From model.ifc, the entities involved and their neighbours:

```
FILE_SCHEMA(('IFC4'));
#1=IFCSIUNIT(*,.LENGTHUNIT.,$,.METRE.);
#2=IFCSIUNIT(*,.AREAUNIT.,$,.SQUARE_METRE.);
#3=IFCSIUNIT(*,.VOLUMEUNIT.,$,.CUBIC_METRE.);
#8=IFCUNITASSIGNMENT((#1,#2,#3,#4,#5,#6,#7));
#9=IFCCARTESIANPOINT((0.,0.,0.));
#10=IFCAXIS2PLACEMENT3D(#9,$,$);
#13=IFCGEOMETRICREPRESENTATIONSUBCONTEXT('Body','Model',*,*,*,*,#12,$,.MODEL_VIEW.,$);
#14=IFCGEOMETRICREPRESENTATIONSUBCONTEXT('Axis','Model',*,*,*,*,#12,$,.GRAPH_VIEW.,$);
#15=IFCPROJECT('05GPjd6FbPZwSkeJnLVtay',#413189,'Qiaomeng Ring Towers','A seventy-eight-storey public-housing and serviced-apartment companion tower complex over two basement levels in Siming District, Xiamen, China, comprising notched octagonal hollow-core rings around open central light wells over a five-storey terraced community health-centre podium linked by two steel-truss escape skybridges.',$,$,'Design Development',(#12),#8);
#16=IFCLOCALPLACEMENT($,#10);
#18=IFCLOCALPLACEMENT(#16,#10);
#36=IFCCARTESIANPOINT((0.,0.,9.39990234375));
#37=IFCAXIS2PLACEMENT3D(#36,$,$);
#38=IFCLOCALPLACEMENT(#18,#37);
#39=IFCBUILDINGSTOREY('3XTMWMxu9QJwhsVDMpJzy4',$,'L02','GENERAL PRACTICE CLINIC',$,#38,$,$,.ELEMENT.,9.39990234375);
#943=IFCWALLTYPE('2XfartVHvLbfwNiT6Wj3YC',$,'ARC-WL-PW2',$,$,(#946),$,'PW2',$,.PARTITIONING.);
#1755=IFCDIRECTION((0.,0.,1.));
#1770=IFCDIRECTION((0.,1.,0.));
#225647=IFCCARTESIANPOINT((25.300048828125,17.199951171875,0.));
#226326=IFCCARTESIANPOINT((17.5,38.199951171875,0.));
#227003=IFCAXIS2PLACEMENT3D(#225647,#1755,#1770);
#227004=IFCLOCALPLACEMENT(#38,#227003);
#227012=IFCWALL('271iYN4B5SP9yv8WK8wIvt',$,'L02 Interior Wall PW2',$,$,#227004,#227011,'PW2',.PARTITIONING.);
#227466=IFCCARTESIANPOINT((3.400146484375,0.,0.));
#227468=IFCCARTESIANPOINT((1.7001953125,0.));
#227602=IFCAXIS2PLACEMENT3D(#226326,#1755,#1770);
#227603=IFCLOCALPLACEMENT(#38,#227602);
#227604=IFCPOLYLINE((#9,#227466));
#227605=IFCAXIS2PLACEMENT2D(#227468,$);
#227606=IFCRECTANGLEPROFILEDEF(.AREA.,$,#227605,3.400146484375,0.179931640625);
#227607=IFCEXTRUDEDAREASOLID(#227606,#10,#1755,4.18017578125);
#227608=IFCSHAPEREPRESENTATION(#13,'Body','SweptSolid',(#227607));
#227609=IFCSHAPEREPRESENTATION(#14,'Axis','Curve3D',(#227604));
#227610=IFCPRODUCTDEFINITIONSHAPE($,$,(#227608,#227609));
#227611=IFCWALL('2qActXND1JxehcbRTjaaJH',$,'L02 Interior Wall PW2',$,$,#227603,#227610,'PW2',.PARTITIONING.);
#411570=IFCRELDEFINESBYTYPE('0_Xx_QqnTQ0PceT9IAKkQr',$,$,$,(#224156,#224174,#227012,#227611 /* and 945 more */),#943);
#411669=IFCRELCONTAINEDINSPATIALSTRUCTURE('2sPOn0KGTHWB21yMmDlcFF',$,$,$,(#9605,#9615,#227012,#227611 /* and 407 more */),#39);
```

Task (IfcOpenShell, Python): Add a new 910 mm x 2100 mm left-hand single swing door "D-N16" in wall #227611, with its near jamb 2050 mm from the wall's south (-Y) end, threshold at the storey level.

```python
import numpy as np
import ifcopenshell
import ifcopenshell.api.feature
import ifcopenshell.api.geometry
import ifcopenshell.api.root
import ifcopenshell.api.spatial
import ifcopenshell.geom
import ifcopenshell.util.element
import ifcopenshell.util.placement
import ifcopenshell.util.representation
import ifcopenshell.util.shape
import ifcopenshell.util.unit

model = ifcopenshell.open("model.ifc")
unit_scale = ifcopenshell.util.unit.calculate_unit_scale(model)
settings = ifcopenshell.geom.settings()


def volume(element):
    """Net volume in cubic metres, openings subtracted."""
    shape = ifcopenshell.geom.create_shape(settings, element)
    return ifcopenshell.util.shape.get_volume(shape.geometry)


wall = model.by_id(227611)
storey = ifcopenshell.util.element.get_container(wall, ifc_class="IfcBuildingStorey")
context = ifcopenshell.util.representation.get_context(model, "Model", "Body", "MODEL_VIEW")
before = volume(wall)

width, height, from_end, sill = 0.91, 2.1, 2.05, 0.0  # metres

# The wall runs along its own X axis, and the end named is its -X end.
wall_shape = ifcopenshell.geom.create_shape(settings, wall)
x, y, z = ifcopenshell.util.shape.get_vertices(wall_shape.geometry).T
start = x.min() + from_end
face, thickness = float(y.min()), float(y.max() - y.min())
wall_matrix = ifcopenshell.util.placement.get_local_placement(wall.ObjectPlacement)
level = ifcopenshell.util.placement.get_local_placement(storey.ObjectPlacement)[2, 3]


def in_wall(x, y):
    """Placement at x, y metres in the wall's axes, at sill height."""
    matrix = wall_matrix.copy()
    matrix[:, 3] = wall_matrix @ np.array([x / unit_scale, y / unit_scale, 0.0, 1.0])
    matrix[2, 3] = level + sill / unit_scale
    return matrix


# Opening: a box that overshoots both wall faces by 50 mm.
opening = ifcopenshell.api.root.create_entity(model, ifc_class="IfcOpeningElement", predefined_type="OPENING")
box = ifcopenshell.api.geometry.add_wall_representation(
    model, context=context, length=width, height=height, thickness=thickness + 0.1
)
ifcopenshell.api.geometry.assign_representation(model, product=opening, representation=box)
ifcopenshell.api.geometry.edit_object_placement(model, product=opening, matrix=in_wall(start, face - 0.05), is_si=False)
ifcopenshell.api.feature.add_feature(model, feature=opening, element=wall)

door = ifcopenshell.api.root.create_entity(model, ifc_class="IfcDoor", name="D-N16", predefined_type="DOOR")
door.OverallWidth, door.OverallHeight = width / unit_scale, height / unit_scale
door.OperationType = "SINGLE_SWING_LEFT"
body = ifcopenshell.api.geometry.add_door_representation(
    model,
    context=context,
    overall_width=door.OverallWidth,
    overall_height=door.OverallHeight,
    operation_type="SINGLE_SWING_LEFT",
    lining_properties={"LiningDepth": thickness / unit_scale, "ThresholdDepth": thickness / unit_scale},
)
ifcopenshell.api.geometry.assign_representation(model, product=door, representation=body)
ifcopenshell.api.spatial.assign_container(model, products=[door], relating_structure=storey)
ifcopenshell.api.feature.add_filling(model, opening=opening, element=door)

# The lining spans the wall, so the door starts at the wall face.
ifcopenshell.api.geometry.edit_object_placement(model, product=door, matrix=in_wall(start, face), is_si=False)

after = volume(wall)

print(f"wall volume {before:.3f} -> {after:.3f} m3")

model.write("model-out.ifc")
```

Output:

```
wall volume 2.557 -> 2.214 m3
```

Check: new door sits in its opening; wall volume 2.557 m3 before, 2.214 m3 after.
